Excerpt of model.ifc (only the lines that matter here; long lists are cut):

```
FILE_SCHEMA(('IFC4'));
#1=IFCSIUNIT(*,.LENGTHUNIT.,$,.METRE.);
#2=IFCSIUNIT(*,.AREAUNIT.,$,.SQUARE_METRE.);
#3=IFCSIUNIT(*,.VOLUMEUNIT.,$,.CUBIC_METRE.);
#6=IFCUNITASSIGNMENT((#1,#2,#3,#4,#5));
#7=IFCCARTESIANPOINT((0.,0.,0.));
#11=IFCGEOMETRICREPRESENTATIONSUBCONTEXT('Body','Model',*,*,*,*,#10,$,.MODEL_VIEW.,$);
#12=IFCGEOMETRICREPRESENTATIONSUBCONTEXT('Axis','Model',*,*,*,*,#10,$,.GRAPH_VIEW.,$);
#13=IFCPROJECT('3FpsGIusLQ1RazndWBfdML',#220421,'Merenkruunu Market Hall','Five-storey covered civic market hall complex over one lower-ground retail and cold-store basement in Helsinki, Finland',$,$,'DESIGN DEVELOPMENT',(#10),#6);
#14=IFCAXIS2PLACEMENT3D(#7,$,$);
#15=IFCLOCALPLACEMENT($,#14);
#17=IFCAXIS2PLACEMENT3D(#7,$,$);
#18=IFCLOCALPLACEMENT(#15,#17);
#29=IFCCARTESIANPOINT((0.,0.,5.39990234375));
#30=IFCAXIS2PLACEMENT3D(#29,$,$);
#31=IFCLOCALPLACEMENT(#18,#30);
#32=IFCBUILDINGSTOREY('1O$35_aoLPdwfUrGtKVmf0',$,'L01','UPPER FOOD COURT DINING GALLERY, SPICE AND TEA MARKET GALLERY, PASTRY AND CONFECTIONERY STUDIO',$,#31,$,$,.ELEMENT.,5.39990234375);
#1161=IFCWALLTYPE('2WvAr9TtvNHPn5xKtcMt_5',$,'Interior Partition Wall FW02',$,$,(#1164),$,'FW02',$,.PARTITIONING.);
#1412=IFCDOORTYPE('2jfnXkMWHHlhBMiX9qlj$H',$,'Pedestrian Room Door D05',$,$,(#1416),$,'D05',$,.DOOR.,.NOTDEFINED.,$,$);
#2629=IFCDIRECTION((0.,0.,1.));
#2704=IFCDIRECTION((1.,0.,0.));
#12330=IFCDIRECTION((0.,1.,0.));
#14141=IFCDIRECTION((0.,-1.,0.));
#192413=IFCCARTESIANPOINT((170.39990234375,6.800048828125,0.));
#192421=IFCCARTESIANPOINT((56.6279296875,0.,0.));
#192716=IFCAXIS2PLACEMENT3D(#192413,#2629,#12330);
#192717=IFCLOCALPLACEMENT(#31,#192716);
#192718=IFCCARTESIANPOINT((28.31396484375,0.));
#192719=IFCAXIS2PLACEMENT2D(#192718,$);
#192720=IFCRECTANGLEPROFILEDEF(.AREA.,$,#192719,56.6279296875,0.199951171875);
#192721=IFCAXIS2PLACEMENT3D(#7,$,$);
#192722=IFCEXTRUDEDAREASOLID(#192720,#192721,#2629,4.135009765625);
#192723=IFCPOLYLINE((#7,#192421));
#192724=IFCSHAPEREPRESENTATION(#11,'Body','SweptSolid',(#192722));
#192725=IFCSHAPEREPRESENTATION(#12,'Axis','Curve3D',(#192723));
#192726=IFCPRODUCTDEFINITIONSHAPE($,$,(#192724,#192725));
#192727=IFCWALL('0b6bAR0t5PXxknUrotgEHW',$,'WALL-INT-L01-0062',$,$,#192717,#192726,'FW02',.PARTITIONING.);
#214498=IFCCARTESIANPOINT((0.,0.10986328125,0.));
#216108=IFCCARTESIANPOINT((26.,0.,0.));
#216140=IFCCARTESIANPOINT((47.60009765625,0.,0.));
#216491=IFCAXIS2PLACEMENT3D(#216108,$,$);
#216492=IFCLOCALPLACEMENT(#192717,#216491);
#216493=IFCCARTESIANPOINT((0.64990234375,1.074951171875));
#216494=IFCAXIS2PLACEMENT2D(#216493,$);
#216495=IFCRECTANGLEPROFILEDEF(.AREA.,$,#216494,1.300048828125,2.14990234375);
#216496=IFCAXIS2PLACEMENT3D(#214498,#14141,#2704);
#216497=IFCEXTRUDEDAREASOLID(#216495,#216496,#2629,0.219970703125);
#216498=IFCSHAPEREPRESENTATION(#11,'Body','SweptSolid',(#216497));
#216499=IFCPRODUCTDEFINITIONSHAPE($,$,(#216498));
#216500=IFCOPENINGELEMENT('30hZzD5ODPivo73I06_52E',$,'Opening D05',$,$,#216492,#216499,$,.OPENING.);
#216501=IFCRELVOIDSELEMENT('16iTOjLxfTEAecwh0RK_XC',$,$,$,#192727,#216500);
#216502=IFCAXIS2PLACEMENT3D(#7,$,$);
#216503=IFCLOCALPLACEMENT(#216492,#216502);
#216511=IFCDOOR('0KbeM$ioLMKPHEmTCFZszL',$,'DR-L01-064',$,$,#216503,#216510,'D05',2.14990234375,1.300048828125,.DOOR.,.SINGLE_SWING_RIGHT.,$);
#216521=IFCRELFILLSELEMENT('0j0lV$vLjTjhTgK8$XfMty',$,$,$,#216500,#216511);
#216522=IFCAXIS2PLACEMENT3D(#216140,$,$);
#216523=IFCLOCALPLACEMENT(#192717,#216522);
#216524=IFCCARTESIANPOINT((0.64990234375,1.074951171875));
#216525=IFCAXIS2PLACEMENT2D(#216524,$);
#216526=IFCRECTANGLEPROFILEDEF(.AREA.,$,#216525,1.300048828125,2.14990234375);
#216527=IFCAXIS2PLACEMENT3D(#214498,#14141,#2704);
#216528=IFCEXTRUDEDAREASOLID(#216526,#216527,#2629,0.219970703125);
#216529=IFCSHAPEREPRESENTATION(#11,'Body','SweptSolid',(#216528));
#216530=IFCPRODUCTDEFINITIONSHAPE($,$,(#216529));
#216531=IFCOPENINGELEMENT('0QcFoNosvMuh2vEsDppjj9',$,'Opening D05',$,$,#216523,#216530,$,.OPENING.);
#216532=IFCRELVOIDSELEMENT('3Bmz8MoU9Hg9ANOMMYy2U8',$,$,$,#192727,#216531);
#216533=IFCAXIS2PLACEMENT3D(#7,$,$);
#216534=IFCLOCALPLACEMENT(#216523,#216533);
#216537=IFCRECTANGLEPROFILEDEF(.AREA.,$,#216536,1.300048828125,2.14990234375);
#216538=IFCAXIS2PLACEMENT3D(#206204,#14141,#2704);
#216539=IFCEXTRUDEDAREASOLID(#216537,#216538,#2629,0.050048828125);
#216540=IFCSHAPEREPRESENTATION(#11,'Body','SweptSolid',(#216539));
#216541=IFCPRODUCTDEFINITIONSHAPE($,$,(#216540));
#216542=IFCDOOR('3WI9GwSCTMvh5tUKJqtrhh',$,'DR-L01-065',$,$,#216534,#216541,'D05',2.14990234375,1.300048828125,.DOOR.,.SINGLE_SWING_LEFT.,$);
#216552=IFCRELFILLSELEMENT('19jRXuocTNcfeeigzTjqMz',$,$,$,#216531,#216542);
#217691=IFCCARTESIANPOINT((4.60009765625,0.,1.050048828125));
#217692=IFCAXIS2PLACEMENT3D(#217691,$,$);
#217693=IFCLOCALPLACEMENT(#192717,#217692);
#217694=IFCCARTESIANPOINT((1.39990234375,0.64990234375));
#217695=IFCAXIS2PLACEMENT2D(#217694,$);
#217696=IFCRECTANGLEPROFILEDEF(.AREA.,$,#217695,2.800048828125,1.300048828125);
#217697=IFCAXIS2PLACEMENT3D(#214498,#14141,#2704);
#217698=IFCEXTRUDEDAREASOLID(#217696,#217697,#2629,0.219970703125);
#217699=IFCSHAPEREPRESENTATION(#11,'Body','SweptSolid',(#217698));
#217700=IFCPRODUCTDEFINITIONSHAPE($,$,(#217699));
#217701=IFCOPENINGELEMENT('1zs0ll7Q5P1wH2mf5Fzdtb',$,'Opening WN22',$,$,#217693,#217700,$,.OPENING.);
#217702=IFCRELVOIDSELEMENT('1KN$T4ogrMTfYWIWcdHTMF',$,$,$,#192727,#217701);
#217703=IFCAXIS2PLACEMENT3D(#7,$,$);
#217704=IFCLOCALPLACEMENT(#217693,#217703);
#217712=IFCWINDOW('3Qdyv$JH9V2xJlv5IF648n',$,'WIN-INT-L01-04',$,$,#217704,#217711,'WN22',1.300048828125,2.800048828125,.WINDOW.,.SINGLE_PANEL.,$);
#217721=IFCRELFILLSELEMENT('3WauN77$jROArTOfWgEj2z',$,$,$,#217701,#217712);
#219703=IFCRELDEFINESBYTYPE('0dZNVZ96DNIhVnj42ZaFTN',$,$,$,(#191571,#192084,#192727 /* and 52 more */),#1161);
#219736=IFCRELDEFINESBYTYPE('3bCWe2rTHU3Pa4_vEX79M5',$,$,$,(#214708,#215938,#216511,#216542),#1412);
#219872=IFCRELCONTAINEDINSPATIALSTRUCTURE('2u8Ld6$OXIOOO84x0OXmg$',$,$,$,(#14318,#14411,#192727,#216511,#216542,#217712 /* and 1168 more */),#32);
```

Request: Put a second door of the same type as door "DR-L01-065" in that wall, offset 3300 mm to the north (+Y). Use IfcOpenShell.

```python
import ifcopenshell
import ifcopenshell.api.feature
import ifcopenshell.api.geometry
import ifcopenshell.api.root
import ifcopenshell.geom
import ifcopenshell.util.element
import ifcopenshell.util.placement
import ifcopenshell.util.shape
import ifcopenshell.util.unit

model = ifcopenshell.open("model.ifc")
unit_scale = ifcopenshell.util.unit.calculate_unit_scale(model)
settings = ifcopenshell.geom.settings()


def volume(element):
    """Net volume in cubic metres, openings subtracted."""
    shape = ifcopenshell.geom.create_shape(settings, element)
    return ifcopenshell.util.shape.get_volume(shape.geometry)


door = model.by_guid("3WI9GwSCTMvh5tUKJqtrhh")
opening = door.FillsVoids[0].RelatingOpeningElement
wall = opening.VoidsElements[0].RelatingBuildingElement
before = volume(wall)
shift = ifcopenshell.util.placement.get_local_placement(wall.ObjectPlacement)[:3, 0] * 3.3 / unit_scale

# copy_class copies the void relationship, type, container and properties, but no geometry.
new_opening = ifcopenshell.api.root.copy_class(model, product=opening)
new_opening.Representation = ifcopenshell.util.element.copy_deep(
    model, opening.Representation, exclude=["IfcGeometricRepresentationContext", "IfcRepresentationMap"]
)
new_door = ifcopenshell.api.root.copy_class(model, product=door)
new_door.Representation = ifcopenshell.util.element.copy_deep(
    model, door.Representation, exclude=["IfcGeometricRepresentationContext", "IfcRepresentationMap"]
)
new_door.Tag = None
ifcopenshell.api.feature.add_filling(model, opening=new_opening, element=new_door)

for old, new in ((opening, new_opening), (door, new_door)):
    matrix = ifcopenshell.util.placement.get_local_placement(old.ObjectPlacement)
    matrix[:3, 3] += shift
    ifcopenshell.api.geometry.edit_object_placement(model, product=new, matrix=matrix, is_si=False)

after = volume(wall)

print(f"wall volume {before:.3f} -> {after:.3f} m3")

model.write("model-out.ifc")
```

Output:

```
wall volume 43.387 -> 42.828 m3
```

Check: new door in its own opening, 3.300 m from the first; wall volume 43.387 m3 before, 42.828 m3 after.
